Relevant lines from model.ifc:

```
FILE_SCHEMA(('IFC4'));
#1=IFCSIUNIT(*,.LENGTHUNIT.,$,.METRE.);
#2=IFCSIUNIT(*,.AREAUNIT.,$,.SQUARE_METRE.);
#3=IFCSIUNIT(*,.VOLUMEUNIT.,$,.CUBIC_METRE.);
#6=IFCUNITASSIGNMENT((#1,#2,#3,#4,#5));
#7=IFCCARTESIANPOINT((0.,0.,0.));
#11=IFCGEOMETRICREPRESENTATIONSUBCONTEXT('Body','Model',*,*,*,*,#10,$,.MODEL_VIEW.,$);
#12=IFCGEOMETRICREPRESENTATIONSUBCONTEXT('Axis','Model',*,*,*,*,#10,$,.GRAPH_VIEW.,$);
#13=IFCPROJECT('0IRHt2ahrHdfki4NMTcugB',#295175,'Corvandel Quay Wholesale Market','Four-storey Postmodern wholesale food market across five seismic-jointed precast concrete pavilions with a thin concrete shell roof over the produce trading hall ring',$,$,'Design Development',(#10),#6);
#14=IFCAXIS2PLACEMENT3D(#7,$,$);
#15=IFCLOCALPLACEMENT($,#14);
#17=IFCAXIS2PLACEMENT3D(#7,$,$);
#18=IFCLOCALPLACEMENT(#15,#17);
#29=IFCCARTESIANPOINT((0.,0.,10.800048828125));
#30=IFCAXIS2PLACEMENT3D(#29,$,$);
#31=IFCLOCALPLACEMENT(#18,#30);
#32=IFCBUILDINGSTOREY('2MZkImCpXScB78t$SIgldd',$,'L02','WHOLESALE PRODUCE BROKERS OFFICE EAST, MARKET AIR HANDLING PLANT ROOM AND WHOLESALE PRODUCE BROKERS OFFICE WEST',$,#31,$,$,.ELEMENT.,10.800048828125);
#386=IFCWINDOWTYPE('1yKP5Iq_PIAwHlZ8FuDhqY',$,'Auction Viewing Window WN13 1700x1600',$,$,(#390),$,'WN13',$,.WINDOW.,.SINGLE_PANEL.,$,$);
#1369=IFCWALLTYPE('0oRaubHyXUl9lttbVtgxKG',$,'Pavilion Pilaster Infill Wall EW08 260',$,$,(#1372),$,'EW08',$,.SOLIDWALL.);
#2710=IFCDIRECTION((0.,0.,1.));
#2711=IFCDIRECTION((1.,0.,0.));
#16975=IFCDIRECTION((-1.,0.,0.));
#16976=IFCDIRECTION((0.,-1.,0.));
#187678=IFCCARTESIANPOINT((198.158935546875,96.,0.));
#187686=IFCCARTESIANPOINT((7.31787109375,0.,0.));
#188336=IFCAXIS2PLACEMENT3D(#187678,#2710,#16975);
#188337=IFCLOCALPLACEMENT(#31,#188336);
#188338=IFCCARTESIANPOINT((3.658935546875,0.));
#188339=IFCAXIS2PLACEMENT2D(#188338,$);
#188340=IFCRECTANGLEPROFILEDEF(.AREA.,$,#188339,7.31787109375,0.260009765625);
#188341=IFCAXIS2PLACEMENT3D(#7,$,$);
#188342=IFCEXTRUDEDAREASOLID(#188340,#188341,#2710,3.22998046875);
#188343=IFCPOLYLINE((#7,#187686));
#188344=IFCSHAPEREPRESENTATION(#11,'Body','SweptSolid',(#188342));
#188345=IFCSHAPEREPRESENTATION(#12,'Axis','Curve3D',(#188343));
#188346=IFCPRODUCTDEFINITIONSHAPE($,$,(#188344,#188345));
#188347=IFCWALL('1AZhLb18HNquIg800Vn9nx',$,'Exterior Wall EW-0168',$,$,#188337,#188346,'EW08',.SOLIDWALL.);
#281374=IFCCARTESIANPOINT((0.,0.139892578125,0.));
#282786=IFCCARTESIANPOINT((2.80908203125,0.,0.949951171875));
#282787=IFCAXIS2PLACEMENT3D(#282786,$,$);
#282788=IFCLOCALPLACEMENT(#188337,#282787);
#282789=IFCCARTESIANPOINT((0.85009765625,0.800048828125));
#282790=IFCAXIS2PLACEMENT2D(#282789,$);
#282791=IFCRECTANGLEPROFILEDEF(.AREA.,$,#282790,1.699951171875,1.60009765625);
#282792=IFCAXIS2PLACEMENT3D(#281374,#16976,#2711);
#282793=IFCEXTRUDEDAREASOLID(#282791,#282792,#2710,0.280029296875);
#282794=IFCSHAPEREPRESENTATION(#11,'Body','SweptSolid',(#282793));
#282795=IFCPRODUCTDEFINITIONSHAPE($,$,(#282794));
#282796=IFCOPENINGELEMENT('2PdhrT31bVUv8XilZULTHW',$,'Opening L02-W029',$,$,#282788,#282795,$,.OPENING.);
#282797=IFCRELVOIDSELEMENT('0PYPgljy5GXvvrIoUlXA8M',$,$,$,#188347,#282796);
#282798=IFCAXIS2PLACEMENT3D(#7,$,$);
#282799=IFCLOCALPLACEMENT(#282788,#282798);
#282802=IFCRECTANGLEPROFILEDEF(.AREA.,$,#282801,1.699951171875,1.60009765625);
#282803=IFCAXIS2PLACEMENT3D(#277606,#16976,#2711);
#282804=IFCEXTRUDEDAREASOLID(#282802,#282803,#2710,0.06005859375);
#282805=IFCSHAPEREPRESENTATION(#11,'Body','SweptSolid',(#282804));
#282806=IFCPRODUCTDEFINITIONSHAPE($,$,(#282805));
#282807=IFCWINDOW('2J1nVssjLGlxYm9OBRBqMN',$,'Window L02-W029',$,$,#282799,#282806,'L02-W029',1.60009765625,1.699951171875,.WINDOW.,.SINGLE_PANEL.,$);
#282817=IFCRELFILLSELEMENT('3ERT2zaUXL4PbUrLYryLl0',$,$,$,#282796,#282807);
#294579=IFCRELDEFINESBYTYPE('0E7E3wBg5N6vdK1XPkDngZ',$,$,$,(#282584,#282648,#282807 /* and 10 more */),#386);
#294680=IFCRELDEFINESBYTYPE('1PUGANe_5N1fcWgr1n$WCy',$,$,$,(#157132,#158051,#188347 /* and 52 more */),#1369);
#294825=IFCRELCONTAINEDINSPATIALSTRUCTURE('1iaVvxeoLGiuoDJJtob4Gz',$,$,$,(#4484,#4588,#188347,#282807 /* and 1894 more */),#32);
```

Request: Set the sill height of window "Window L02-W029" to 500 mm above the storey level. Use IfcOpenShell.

```python
import numpy as np
import ifcopenshell
import ifcopenshell.api.geometry
import ifcopenshell.geom
import ifcopenshell.util.element
import ifcopenshell.util.placement
import ifcopenshell.util.shape
import ifcopenshell.util.unit

model = ifcopenshell.open("model.ifc")
unit_scale = ifcopenshell.util.unit.calculate_unit_scale(model)

window = model.by_guid("2J1nVssjLGlxYm9OBRBqMN")
opening = window.FillsVoids[0].RelatingOpeningElement
storey = ifcopenshell.util.element.get_container(window, ifc_class="IfcBuildingStorey")
level = ifcopenshell.util.placement.get_local_placement(storey.ObjectPlacement)[2, 3]

# The opening's origin need not be at the sill, so measure its lowest point.
shape = ifcopenshell.geom.create_shape(ifcopenshell.geom.settings(), opening)
bottom = ifcopenshell.util.shape.get_shape_bottom_elevation(shape, shape.geometry) / unit_scale
dz = level + 0.5 - bottom

shift = np.array([0.0, 0.0, dz])
# The window is placed relative to its opening, so it follows when the opening moves.
matrix = ifcopenshell.util.placement.get_local_placement(opening.ObjectPlacement)
matrix[:3, 3] += shift
ifcopenshell.api.geometry.edit_object_placement(
    model, product=opening, matrix=matrix, is_si=False, should_transform_children=True
)

print(f"moved by {dz * unit_scale:+.3f} m")

model.write("model_updated.ifc")
```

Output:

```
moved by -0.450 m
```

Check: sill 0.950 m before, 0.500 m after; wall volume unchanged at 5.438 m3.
